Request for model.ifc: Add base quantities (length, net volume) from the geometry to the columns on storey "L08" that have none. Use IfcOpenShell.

First a look at what the model holds.

```python
import ifcopenshell
import ifcopenshell.util.element
import ifcopenshell.util.unit

model = ifcopenshell.open("model.ifc")
print(model.schema)
for unit_type in ("LENGTHUNIT", "AREAUNIT", "VOLUMEUNIT"):
    print(unit_type, ifcopenshell.util.unit.calculate_unit_scale(model, unit_type))
storey = next(s for s in model.by_type("IfcBuildingStorey") if s.Name == "L08")
columns = [e for e in ifcopenshell.util.element.get_decomposition(storey) if e.is_a("IfcColumn")]
for e in sorted(columns, key=lambda e: e.id()):
    print(e.id(), e.is_a(), e.Name, list(ifcopenshell.util.element.get_psets(e, qtos_only=True)), sep=" | ")
```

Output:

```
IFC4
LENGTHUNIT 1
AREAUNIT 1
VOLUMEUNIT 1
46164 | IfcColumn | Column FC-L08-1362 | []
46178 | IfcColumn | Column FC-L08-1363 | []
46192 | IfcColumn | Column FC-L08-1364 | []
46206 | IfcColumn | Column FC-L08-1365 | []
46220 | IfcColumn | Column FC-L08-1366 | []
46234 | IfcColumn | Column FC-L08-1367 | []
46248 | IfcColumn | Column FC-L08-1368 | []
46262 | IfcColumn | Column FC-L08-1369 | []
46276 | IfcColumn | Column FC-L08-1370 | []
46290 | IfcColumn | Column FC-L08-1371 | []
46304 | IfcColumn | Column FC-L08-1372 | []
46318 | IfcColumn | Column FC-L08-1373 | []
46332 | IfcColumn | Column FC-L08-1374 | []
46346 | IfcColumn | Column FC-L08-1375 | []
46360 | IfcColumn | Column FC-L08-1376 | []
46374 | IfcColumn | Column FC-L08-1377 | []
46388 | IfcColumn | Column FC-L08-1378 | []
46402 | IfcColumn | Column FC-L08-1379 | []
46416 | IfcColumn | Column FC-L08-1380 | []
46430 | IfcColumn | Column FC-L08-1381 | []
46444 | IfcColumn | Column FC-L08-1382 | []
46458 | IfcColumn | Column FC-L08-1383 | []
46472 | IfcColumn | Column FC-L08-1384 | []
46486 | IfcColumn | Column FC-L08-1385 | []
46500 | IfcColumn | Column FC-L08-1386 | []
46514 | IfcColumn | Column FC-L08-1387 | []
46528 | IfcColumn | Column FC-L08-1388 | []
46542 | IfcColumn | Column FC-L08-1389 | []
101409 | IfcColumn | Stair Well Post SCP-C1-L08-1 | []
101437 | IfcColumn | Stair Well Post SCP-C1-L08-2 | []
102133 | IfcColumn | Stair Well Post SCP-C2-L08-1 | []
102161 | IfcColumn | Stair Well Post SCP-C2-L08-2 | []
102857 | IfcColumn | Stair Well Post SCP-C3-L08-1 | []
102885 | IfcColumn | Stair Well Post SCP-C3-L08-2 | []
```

```python
import ifcopenshell
import ifcopenshell.api.pset
import ifcopenshell.geom
import ifcopenshell.util.element
import ifcopenshell.util.shape
import ifcopenshell.util.unit

model = ifcopenshell.open("model.ifc")
unit_scale = ifcopenshell.util.unit.calculate_unit_scale(model)
volume_scale = ifcopenshell.util.unit.calculate_unit_scale(model, "VOLUMEUNIT")
settings = ifcopenshell.geom.settings()

storey = next(s for s in model.by_type("IfcBuildingStorey") if s.Name == "L08")
columns = [e for e in ifcopenshell.util.element.get_decomposition(storey) if e.is_a("IfcColumn")]

for e in sorted(columns, key=lambda e: e.id()):
    if ifcopenshell.util.element.get_psets(e, qtos_only=True, should_inherit=False):
        continue
    # Geometry comes back in metres, in the element's own axes.
    shape = ifcopenshell.geom.create_shape(settings, e)
    values = {
        "Length": ifcopenshell.util.shape.get_z(shape.geometry) / unit_scale,
        "NetVolume": ifcopenshell.util.shape.get_volume(shape.geometry) / volume_scale,
    }
    qto = ifcopenshell.api.pset.add_qto(model, product=e, name="Qto_ColumnBaseQuantities")
    ifcopenshell.api.pset.edit_qto(model, qto=qto, properties=values)
    print(e.id(), {k: round(v, 3) for k, v in values.items()})

model.write("model_v2.ifc")
```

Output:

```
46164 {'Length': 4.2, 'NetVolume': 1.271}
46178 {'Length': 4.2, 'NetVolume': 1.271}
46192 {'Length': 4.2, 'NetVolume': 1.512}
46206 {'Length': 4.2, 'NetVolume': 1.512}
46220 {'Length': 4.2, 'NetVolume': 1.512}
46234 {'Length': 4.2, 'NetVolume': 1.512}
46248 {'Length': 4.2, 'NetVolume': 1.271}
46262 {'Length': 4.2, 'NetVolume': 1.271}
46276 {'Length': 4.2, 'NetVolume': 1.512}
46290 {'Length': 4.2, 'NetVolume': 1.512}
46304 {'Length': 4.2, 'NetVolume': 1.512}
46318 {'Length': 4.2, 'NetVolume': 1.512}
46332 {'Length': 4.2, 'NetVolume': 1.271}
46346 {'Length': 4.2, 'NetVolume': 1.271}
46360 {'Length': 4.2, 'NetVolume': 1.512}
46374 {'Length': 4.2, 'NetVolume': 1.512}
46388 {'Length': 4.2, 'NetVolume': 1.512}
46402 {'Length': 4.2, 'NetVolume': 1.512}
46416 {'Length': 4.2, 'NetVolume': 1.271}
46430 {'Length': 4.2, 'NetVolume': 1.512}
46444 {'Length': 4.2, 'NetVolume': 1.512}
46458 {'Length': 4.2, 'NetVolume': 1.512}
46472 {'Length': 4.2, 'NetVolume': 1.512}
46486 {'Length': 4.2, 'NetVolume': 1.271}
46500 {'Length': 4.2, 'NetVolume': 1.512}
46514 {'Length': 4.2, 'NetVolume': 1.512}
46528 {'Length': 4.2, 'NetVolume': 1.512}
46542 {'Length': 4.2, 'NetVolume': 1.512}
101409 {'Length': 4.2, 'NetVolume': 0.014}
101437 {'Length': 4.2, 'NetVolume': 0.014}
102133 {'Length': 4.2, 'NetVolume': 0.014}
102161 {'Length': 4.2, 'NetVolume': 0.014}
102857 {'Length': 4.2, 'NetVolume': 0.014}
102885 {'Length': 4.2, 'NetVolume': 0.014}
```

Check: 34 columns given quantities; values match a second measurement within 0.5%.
